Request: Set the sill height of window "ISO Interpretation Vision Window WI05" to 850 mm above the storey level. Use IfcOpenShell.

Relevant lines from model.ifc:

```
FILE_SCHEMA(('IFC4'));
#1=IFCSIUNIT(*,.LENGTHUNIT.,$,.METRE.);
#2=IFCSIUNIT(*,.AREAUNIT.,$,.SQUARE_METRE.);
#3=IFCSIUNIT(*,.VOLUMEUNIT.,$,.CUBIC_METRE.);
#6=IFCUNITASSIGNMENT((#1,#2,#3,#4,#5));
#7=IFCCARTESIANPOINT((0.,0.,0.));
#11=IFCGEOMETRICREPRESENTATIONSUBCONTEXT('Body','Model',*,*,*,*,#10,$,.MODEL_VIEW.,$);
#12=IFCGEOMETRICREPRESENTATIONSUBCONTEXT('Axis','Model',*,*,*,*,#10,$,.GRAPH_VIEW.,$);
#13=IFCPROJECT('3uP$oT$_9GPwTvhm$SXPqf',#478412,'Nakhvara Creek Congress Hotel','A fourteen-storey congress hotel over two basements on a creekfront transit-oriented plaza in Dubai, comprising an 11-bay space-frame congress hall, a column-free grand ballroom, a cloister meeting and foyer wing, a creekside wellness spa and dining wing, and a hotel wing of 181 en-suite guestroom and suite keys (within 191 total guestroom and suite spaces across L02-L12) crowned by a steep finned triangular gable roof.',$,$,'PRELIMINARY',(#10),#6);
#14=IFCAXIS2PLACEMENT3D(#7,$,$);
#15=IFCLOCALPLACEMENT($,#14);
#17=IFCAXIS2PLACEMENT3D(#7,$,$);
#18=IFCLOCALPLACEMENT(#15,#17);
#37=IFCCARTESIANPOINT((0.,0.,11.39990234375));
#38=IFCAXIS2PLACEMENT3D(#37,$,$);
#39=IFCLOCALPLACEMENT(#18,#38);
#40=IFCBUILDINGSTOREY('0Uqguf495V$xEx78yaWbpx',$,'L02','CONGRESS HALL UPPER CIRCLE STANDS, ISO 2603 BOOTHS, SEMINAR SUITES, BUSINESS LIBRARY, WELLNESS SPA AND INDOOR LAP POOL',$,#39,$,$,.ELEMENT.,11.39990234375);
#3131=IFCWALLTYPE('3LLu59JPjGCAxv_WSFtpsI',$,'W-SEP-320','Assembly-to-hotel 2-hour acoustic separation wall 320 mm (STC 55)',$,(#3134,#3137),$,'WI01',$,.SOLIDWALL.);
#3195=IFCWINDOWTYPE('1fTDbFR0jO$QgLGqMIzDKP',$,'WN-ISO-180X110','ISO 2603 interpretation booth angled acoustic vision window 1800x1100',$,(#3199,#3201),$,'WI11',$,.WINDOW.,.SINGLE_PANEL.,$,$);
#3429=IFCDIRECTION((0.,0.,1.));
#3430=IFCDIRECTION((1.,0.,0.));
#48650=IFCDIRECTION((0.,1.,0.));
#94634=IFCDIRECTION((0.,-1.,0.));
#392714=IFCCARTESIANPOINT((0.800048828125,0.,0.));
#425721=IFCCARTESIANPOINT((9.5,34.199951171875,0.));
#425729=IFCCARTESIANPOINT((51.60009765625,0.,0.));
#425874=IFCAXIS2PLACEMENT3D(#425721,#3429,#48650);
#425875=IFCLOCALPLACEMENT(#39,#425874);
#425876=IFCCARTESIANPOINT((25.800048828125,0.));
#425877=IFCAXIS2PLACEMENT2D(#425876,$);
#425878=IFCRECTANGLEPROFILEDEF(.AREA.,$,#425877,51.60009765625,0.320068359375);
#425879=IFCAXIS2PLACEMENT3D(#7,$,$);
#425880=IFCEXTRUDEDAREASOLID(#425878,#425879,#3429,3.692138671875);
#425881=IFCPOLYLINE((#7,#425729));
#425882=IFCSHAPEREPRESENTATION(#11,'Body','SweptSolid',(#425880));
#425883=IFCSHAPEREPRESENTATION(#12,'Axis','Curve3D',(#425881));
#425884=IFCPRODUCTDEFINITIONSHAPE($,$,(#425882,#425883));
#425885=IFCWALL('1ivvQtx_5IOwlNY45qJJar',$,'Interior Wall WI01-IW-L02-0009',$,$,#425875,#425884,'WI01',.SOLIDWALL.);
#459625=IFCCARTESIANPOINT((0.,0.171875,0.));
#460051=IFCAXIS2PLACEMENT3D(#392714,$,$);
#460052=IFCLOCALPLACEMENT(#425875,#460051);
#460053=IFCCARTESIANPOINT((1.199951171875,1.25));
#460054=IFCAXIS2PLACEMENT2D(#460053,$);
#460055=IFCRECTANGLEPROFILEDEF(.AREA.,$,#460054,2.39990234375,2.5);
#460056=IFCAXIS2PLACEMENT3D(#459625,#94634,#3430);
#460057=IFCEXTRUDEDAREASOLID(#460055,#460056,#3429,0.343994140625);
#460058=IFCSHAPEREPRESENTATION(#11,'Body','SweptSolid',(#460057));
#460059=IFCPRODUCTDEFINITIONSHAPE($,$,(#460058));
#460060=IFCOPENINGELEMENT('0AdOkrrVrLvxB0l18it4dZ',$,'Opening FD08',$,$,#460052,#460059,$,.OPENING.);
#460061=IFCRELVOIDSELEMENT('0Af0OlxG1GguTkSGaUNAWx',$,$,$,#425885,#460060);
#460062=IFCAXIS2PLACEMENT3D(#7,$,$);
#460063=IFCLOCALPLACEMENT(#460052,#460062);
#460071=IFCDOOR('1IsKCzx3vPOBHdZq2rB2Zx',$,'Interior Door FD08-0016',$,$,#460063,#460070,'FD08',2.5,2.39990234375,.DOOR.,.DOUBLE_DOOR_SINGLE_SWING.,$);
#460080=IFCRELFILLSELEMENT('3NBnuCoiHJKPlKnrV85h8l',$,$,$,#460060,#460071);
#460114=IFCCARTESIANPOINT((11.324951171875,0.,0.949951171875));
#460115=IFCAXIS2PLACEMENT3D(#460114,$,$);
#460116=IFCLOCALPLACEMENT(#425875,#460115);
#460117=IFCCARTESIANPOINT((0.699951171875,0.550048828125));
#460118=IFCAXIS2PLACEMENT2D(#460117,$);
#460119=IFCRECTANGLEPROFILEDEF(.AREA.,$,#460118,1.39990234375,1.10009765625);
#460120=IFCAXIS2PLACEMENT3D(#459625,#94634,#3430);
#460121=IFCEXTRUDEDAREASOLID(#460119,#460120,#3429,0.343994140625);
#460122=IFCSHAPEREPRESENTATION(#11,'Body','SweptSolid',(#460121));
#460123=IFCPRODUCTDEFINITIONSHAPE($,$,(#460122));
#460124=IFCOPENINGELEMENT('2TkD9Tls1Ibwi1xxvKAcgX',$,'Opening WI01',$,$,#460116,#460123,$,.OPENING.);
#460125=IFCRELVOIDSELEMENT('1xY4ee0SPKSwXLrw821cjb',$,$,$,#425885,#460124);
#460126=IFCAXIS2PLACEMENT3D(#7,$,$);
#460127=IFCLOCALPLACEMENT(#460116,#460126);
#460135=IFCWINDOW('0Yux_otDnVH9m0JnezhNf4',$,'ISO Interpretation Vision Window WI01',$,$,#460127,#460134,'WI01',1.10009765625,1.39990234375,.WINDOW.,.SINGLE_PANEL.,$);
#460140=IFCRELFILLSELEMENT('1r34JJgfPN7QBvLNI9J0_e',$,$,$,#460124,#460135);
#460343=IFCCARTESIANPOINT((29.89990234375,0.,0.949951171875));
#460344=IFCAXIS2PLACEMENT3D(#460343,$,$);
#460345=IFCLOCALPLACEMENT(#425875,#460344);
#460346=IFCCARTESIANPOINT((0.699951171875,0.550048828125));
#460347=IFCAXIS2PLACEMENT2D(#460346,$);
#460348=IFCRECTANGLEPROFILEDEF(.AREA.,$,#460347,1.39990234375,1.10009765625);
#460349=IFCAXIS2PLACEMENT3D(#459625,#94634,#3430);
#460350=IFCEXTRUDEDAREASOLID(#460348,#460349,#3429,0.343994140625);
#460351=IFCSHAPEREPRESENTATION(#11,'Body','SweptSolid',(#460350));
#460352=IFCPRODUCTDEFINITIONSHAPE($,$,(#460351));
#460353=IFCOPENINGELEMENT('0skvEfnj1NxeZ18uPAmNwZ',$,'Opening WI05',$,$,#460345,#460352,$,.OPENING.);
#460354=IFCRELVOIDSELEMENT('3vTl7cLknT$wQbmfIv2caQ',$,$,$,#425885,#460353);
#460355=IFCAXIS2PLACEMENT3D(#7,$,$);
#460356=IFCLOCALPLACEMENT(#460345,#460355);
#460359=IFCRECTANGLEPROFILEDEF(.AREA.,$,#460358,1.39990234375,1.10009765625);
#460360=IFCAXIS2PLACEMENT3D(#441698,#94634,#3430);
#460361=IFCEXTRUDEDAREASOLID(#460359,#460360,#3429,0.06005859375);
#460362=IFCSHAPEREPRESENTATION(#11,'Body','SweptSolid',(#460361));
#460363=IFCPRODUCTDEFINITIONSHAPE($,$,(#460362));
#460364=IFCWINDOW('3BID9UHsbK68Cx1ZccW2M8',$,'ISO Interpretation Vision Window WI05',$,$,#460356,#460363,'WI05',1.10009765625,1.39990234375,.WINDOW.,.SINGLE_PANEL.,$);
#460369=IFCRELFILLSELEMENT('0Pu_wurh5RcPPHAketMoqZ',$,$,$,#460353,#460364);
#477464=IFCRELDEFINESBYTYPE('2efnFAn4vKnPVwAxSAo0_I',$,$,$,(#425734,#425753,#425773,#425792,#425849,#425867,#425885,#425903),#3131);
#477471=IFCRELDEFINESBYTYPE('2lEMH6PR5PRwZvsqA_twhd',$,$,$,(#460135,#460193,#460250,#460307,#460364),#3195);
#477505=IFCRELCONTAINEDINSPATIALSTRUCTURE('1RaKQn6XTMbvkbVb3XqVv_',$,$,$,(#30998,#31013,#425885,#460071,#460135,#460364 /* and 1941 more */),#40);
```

```python
import numpy as np
import ifcopenshell
import ifcopenshell.api.geometry
import ifcopenshell.geom
import ifcopenshell.util.element
import ifcopenshell.util.placement
import ifcopenshell.util.shape
import ifcopenshell.util.unit

model = ifcopenshell.open("model.ifc")
unit_scale = ifcopenshell.util.unit.calculate_unit_scale(model)

window = model.by_guid("3BID9UHsbK68Cx1ZccW2M8")
opening = window.FillsVoids[0].RelatingOpeningElement
storey = ifcopenshell.util.element.get_container(window, ifc_class="IfcBuildingStorey")
level = ifcopenshell.util.placement.get_local_placement(storey.ObjectPlacement)[2, 3]

# The opening's origin need not be at the sill, so measure its lowest point.
shape = ifcopenshell.geom.create_shape(ifcopenshell.geom.settings(), opening)
bottom = ifcopenshell.util.shape.get_shape_bottom_elevation(shape, shape.geometry) / unit_scale
dz = level + 0.85 - bottom

shift = np.array([0.0, 0.0, dz])
# The window is placed relative to its opening, so it follows when the opening moves.
matrix = ifcopenshell.util.placement.get_local_placement(opening.ObjectPlacement)
matrix[:3, 3] += shift
ifcopenshell.api.geometry.edit_object_placement(
    model, product=opening, matrix=matrix, is_si=False, should_transform_children=True
)

print(f"moved by {dz * unit_scale:+.3f} m")

model.write("model_rev.ifc")
```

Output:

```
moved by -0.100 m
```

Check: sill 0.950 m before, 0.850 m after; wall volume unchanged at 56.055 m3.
